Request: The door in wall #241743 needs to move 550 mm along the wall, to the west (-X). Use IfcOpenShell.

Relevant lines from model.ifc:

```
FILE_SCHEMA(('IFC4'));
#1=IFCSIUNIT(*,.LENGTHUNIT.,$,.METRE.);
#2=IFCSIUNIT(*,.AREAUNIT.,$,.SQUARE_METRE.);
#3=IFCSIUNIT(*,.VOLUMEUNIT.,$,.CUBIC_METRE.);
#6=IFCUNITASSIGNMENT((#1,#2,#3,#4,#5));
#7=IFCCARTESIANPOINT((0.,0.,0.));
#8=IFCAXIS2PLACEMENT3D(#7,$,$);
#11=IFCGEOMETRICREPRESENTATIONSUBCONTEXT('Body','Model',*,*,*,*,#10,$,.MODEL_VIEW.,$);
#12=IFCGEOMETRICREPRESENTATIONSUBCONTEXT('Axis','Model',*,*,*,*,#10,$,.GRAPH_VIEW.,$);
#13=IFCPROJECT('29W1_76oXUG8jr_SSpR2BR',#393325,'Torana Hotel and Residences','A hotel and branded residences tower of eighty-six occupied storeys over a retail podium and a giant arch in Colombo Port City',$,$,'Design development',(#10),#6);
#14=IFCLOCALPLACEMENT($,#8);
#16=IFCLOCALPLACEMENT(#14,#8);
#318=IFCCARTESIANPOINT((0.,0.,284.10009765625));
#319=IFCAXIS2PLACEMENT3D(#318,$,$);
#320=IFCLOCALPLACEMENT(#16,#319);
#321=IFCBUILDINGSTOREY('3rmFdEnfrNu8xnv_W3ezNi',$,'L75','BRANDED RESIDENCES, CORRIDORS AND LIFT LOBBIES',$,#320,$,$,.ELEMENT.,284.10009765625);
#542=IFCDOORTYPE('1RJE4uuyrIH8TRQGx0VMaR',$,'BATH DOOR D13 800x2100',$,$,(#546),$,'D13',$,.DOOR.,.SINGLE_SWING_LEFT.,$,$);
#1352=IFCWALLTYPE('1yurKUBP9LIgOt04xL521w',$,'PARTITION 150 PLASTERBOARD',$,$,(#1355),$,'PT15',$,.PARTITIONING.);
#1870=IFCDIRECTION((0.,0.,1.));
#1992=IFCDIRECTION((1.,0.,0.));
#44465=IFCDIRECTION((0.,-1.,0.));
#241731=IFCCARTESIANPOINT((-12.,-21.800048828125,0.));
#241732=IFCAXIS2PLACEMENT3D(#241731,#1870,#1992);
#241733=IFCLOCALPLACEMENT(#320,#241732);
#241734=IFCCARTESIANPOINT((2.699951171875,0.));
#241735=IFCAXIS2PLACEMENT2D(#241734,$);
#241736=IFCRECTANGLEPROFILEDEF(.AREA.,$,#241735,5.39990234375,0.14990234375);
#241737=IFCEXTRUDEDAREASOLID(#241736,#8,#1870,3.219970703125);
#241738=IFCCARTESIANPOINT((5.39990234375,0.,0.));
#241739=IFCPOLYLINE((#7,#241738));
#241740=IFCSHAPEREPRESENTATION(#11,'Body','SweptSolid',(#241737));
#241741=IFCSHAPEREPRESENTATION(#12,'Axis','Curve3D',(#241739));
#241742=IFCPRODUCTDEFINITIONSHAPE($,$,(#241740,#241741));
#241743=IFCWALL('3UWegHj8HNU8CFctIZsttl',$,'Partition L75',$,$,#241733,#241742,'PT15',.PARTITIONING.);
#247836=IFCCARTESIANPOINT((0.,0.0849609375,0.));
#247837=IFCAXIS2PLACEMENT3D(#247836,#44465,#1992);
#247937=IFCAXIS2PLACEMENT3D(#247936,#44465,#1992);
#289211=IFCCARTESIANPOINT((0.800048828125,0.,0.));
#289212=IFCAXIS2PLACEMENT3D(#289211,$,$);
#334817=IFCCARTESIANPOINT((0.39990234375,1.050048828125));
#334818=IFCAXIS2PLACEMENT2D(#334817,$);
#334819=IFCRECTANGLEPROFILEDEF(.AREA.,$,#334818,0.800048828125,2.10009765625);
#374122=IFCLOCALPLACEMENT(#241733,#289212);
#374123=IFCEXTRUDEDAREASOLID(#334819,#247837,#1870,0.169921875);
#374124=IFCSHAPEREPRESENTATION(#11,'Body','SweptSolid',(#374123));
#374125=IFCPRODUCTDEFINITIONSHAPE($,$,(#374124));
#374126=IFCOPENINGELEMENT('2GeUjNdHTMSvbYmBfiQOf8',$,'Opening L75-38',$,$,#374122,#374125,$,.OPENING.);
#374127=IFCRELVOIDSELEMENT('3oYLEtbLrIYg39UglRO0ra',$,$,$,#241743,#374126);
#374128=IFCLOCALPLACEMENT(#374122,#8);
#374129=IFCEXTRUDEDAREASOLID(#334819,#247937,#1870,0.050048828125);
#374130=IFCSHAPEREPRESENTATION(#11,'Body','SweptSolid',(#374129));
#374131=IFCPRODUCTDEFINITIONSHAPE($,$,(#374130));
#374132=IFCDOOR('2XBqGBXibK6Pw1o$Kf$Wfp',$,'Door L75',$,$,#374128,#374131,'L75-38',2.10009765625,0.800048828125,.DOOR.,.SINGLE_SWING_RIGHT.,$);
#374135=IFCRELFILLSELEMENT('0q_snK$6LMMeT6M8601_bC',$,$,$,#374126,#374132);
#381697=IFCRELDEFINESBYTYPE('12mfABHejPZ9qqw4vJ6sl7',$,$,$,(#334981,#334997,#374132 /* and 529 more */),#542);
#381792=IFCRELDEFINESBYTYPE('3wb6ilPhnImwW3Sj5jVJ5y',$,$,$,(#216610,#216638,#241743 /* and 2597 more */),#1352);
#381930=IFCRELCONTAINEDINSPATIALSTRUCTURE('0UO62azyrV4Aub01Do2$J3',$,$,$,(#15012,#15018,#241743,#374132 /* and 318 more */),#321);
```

```python
import ifcopenshell
import ifcopenshell.api.geometry
import ifcopenshell.util.placement
import ifcopenshell.util.unit

model = ifcopenshell.open("model.ifc")
unit_scale = ifcopenshell.util.unit.calculate_unit_scale(model)

door = model.by_guid("2XBqGBXibK6Pw1o$Kf$Wfp")
opening = door.FillsVoids[0].RelatingOpeningElement
wall = opening.VoidsElements[0].RelatingBuildingElement

wall_matrix = ifcopenshell.util.placement.get_local_placement(wall.ObjectPlacement)
shift = wall_matrix[:3, 0] * -0.55 / unit_scale
before = ifcopenshell.util.placement.get_local_placement(door.ObjectPlacement)[:3, 3].copy()

# The door is placed relative to its opening, so it follows when the opening moves.
matrix = ifcopenshell.util.placement.get_local_placement(opening.ObjectPlacement)
matrix[:3, 3] += shift
ifcopenshell.api.geometry.edit_object_placement(
    model, product=opening, matrix=matrix, is_si=False, should_transform_children=True
)

after = ifcopenshell.util.placement.get_local_placement(door.ObjectPlacement)[:3, 3]
print("door moved by", (after - before).round(3) + 0.0)

model.write("model_edited.ifc")
```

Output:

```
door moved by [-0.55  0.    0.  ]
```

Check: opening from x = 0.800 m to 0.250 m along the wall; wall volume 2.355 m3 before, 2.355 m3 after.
